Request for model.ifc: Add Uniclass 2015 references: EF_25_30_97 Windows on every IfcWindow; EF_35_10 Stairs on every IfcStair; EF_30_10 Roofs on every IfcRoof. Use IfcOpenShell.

First a look at what the model holds.

```python
import ifcopenshell

model = ifcopenshell.open("model.ifc")
print(model.schema)
print("classifications:", [c.Name for c in model.by_type("IfcClassification")])
for ifc_class in ("IfcDoor", "IfcRoof", "IfcStair", "IfcWall", "IfcWindow"):
    print(ifc_class, len(model.by_type(ifc_class)))
```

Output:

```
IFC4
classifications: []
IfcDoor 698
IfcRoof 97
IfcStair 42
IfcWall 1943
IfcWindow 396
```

```python
import ifcopenshell
import ifcopenshell.api.classification

model = ifcopenshell.open("model.ifc")

system = ifcopenshell.api.classification.add_classification(model, classification="Uniclass 2015")

codes = {
    "IfcWindow": ("EF_25_30_97", "Windows"),
    "IfcStair": ("EF_35_10", "Stairs"),
    "IfcRoof": ("EF_30_10", "Roofs"),
}
for ifc_class, (code, name) in codes.items():
    products = model.by_type(ifc_class)
    ifcopenshell.api.classification.add_reference(
        model, products=products, classification=system, identification=code, name=name
    )
    print(code, len(products))

model.write("model_updated.ifc")
```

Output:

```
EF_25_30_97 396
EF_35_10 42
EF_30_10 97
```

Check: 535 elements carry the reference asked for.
